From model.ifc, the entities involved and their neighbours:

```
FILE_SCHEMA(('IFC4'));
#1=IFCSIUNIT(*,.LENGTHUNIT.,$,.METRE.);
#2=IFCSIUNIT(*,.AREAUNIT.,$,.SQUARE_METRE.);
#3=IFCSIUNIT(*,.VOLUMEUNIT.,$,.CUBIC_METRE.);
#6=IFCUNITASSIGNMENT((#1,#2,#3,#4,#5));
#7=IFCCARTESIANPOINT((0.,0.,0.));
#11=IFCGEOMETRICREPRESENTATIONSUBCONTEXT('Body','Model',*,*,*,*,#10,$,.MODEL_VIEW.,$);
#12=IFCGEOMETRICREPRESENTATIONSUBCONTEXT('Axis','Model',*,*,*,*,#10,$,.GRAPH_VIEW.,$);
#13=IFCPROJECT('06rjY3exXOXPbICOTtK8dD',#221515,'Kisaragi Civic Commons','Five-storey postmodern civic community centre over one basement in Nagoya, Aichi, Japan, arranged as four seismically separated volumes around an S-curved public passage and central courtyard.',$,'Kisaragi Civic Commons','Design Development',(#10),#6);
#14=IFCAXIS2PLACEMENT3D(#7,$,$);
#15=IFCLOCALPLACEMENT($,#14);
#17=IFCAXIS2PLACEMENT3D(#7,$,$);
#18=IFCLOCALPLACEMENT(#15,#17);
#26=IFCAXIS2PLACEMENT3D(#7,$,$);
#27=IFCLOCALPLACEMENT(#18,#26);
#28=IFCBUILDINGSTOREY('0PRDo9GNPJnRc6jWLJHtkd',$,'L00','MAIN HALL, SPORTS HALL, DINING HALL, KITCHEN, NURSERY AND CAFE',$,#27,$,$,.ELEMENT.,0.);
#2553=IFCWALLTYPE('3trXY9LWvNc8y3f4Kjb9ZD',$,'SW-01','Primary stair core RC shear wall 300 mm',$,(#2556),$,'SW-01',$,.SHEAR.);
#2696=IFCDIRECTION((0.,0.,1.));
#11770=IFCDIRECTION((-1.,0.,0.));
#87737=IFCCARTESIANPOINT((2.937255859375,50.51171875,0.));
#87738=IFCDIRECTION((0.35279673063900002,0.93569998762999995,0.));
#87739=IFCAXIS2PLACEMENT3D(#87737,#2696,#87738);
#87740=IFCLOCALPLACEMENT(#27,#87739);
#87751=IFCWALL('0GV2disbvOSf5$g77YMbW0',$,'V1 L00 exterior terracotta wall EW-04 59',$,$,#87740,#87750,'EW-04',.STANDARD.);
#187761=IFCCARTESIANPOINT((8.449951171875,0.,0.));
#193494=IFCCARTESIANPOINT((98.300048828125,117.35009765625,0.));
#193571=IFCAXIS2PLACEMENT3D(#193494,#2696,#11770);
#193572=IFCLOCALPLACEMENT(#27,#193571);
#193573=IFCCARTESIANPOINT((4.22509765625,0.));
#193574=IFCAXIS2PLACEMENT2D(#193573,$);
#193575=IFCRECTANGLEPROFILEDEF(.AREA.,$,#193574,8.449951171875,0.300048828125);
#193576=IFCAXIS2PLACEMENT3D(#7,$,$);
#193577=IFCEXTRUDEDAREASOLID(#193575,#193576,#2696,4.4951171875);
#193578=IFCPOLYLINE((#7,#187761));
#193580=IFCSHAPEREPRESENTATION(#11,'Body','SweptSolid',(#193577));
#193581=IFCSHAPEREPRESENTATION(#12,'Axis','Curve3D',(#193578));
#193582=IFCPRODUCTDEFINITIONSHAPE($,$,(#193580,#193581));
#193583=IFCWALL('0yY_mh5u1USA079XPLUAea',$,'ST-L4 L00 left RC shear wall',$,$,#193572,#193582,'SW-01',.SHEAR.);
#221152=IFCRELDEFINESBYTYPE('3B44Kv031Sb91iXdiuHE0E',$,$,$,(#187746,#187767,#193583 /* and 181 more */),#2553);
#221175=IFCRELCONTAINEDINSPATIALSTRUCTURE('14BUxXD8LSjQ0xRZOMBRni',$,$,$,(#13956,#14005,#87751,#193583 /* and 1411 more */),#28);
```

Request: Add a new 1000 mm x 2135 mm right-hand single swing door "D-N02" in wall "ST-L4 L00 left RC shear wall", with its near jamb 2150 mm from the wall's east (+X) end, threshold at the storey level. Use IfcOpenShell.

```python
import numpy as np
import ifcopenshell
import ifcopenshell.api.feature
import ifcopenshell.api.geometry
import ifcopenshell.api.root
import ifcopenshell.api.spatial
import ifcopenshell.geom
import ifcopenshell.util.element
import ifcopenshell.util.placement
import ifcopenshell.util.representation
import ifcopenshell.util.shape
import ifcopenshell.util.unit

model = ifcopenshell.open("model.ifc")
unit_scale = ifcopenshell.util.unit.calculate_unit_scale(model)
settings = ifcopenshell.geom.settings()


def volume(element):
    """Net volume in cubic metres, openings subtracted."""
    shape = ifcopenshell.geom.create_shape(settings, element)
    return ifcopenshell.util.shape.get_volume(shape.geometry)


wall = model.by_guid("0yY_mh5u1USA079XPLUAea")
storey = ifcopenshell.util.element.get_container(wall, ifc_class="IfcBuildingStorey")
context = ifcopenshell.util.representation.get_context(model, "Model", "Body", "MODEL_VIEW")
before = volume(wall)

width, height, from_end, sill = 1, 2.135, 2.15, 0.0  # metres

# The wall runs along its own X axis, and the end named is its -X end.
wall_shape = ifcopenshell.geom.create_shape(settings, wall)
x, y, z = ifcopenshell.util.shape.get_vertices(wall_shape.geometry).T
start = x.min() + from_end
face, thickness = float(y.min()), float(y.max() - y.min())
wall_matrix = ifcopenshell.util.placement.get_local_placement(wall.ObjectPlacement)
level = ifcopenshell.util.placement.get_local_placement(storey.ObjectPlacement)[2, 3]


def in_wall(x, y):
    """Placement at x, y metres in the wall's axes, at sill height."""
    matrix = wall_matrix.copy()
    matrix[:, 3] = wall_matrix @ np.array([x / unit_scale, y / unit_scale, 0.0, 1.0])
    matrix[2, 3] = level + sill / unit_scale
    return matrix


# Opening: a box that overshoots both wall faces by 50 mm.
opening = ifcopenshell.api.root.create_entity(model, ifc_class="IfcOpeningElement", predefined_type="OPENING")
box = ifcopenshell.api.geometry.add_wall_representation(
    model, context=context, length=width, height=height, thickness=thickness + 0.1
)
ifcopenshell.api.geometry.assign_representation(model, product=opening, representation=box)
ifcopenshell.api.geometry.edit_object_placement(model, product=opening, matrix=in_wall(start, face - 0.05), is_si=False)
ifcopenshell.api.feature.add_feature(model, feature=opening, element=wall)

door = ifcopenshell.api.root.create_entity(model, ifc_class="IfcDoor", name="D-N02", predefined_type="DOOR")
door.OverallWidth, door.OverallHeight = width / unit_scale, height / unit_scale
door.OperationType = "SINGLE_SWING_RIGHT"
body = ifcopenshell.api.geometry.add_door_representation(
    model,
    context=context,
    overall_width=door.OverallWidth,
    overall_height=door.OverallHeight,
    operation_type="SINGLE_SWING_RIGHT",
    lining_properties={"LiningDepth": thickness / unit_scale, "ThresholdDepth": thickness / unit_scale},
)
ifcopenshell.api.geometry.assign_representation(model, product=door, representation=body)
ifcopenshell.api.spatial.assign_container(model, products=[door], relating_structure=storey)
ifcopenshell.api.feature.add_filling(model, opening=opening, element=door)

# The lining spans the wall, so the door starts at the wall face.
ifcopenshell.api.geometry.edit_object_placement(model, product=door, matrix=in_wall(start, face), is_si=False)

after = volume(wall)

print(f"wall volume {before:.3f} -> {after:.3f} m3")

model.write("model-out.ifc")
```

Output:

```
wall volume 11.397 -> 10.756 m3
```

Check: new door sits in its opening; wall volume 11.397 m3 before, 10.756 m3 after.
